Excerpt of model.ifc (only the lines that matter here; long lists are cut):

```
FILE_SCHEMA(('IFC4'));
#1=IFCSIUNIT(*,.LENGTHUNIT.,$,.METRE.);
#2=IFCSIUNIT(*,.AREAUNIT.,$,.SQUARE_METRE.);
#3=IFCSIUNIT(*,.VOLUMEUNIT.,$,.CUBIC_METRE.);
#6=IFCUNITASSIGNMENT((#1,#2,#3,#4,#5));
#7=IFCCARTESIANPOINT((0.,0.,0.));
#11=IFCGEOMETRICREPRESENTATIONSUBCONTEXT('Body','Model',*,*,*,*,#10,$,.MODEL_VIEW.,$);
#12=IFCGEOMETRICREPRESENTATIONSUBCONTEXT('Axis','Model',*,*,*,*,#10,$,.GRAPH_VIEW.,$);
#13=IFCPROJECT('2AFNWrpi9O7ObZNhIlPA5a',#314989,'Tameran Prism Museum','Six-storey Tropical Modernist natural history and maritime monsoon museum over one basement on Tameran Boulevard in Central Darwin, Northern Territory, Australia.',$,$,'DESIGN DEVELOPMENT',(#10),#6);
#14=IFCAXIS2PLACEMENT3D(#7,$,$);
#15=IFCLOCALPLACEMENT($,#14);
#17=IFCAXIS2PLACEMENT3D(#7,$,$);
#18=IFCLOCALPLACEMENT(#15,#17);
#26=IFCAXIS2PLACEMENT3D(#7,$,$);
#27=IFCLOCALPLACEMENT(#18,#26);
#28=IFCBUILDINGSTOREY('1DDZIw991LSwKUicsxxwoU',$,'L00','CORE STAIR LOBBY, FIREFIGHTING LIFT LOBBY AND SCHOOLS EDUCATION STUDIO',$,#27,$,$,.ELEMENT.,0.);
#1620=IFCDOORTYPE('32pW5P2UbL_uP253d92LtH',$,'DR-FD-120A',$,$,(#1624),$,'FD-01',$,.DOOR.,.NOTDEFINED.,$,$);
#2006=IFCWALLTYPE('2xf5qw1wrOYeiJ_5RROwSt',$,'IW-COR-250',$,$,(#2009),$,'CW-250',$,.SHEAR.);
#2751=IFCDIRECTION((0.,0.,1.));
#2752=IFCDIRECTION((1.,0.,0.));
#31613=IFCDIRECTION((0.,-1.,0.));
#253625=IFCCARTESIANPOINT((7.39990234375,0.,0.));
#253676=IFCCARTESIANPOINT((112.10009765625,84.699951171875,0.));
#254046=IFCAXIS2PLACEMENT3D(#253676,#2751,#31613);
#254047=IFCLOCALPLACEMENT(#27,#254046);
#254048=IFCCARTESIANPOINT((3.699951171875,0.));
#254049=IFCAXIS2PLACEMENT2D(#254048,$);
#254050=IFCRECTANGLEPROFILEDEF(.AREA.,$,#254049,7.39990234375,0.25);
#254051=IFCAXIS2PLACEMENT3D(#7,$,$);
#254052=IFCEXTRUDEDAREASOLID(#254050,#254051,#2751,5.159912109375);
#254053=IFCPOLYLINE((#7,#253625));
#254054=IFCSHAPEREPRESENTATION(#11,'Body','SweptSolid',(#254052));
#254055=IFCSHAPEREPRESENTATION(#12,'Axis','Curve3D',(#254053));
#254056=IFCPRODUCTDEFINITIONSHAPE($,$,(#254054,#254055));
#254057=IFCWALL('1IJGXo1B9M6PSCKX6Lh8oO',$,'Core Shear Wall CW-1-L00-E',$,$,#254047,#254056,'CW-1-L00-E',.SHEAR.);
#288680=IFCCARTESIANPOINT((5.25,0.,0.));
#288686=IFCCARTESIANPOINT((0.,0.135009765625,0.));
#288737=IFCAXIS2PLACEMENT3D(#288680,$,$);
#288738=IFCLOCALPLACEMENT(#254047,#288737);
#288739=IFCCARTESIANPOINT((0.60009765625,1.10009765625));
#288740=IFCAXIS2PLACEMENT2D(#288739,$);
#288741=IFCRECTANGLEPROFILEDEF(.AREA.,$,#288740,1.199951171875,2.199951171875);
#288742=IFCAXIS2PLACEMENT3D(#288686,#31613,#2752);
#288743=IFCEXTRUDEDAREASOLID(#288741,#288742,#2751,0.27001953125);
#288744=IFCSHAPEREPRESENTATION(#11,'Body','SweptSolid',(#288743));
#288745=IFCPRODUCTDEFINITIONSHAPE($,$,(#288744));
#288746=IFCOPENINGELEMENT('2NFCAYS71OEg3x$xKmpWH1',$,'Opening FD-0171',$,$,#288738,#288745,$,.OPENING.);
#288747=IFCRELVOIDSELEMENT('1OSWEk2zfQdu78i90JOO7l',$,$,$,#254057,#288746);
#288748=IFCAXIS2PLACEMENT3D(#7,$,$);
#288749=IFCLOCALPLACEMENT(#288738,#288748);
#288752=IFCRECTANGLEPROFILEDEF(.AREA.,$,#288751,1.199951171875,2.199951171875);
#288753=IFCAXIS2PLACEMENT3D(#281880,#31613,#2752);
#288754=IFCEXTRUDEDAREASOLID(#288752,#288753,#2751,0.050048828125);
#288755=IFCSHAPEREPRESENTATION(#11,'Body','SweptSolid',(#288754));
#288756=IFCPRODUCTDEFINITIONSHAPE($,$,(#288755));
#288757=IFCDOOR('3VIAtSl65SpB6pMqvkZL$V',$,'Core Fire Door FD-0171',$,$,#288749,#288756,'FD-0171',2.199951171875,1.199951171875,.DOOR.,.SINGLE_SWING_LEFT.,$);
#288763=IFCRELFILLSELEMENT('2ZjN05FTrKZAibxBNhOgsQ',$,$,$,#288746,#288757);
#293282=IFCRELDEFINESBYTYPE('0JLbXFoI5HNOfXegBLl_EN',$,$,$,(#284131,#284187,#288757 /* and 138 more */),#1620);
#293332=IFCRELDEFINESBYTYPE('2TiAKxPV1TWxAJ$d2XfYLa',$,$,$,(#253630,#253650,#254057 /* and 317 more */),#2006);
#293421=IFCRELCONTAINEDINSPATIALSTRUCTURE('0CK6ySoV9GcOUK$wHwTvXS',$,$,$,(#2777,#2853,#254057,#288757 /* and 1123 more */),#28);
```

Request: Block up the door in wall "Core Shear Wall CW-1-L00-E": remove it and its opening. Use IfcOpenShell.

```python
import ifcopenshell
import ifcopenshell.api.feature
import ifcopenshell.api.root
import ifcopenshell.geom
import ifcopenshell.util.shape

model = ifcopenshell.open("model.ifc")
settings = ifcopenshell.geom.settings()


def volume(element):
    """Net volume in cubic metres, openings subtracted."""
    shape = ifcopenshell.geom.create_shape(settings, element)
    return ifcopenshell.util.shape.get_volume(shape.geometry)


door = model.by_guid("3VIAtSl65SpB6pMqvkZL$V")
opening = door.FillsVoids[0].RelatingOpeningElement
wall = opening.VoidsElements[0].RelatingBuildingElement
before = volume(wall)

ifcopenshell.api.root.remove_product(model, product=door)
ifcopenshell.api.feature.remove_feature(model, feature=opening)

after = volume(wall)

print(f"wall volume {before:.3f} -> {after:.3f} m3")

model.write("model-out.ifc")
```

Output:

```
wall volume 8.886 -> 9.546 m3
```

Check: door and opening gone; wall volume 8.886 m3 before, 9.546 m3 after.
